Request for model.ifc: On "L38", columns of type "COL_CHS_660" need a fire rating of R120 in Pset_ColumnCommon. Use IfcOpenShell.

First a look at what the model holds.

```python
import ifcopenshell
import ifcopenshell.util.element

model = ifcopenshell.open("model.ifc")
print(model.schema)
storey = next(s for s in model.by_type("IfcBuildingStorey") if s.Name == "L38")
columns = [e for e in ifcopenshell.util.element.get_decomposition(storey) if e.is_a("IfcColumn")]
seen = {}
for e in columns:
    element_type = ifcopenshell.util.element.get_type(e)
    key = (element_type.Name if element_type != e and element_type else None, ifcopenshell.util.element.get_pset(e, "Pset_ColumnCommon", "FireRating"))
    seen[key] = seen.get(key, 0) + 1
for (name, value), count in sorted(seen.items(), key=str):
    print(count, "x", name, "|", value)
```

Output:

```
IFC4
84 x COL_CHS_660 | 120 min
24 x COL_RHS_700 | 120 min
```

```python
import ifcopenshell
import ifcopenshell.api.pset
import ifcopenshell.util.element

model = ifcopenshell.open("model.ifc")

storey = next(s for s in model.by_type("IfcBuildingStorey") if s.Name == "L38")
columns = [e for e in ifcopenshell.util.element.get_decomposition(storey) if e.is_a("IfcColumn")]

count = 0
for e in columns:
    element_type = ifcopenshell.util.element.get_type(e)
    if element_type in (None, e) or element_type.Name != "COL_CHS_660":
        continue
    found = ifcopenshell.util.element.get_pset(e, "Pset_ColumnCommon", should_inherit=False)
    if found:
        pset = model.by_id(found["id"])
        if len(ifcopenshell.util.element.get_elements_by_pset(pset)) > 1:
            pset = ifcopenshell.api.pset.unshare_pset(model, products=[e], pset=pset)[0]
    else:
        pset = ifcopenshell.api.pset.add_pset(model, product=e, name="Pset_ColumnCommon")
    ifcopenshell.api.pset.edit_pset(model, pset=pset, properties={"FireRating": "R120"})
    count += 1

print(count, "columns updated")

model.write("model_v2.ifc")
```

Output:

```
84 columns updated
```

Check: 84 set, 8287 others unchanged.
